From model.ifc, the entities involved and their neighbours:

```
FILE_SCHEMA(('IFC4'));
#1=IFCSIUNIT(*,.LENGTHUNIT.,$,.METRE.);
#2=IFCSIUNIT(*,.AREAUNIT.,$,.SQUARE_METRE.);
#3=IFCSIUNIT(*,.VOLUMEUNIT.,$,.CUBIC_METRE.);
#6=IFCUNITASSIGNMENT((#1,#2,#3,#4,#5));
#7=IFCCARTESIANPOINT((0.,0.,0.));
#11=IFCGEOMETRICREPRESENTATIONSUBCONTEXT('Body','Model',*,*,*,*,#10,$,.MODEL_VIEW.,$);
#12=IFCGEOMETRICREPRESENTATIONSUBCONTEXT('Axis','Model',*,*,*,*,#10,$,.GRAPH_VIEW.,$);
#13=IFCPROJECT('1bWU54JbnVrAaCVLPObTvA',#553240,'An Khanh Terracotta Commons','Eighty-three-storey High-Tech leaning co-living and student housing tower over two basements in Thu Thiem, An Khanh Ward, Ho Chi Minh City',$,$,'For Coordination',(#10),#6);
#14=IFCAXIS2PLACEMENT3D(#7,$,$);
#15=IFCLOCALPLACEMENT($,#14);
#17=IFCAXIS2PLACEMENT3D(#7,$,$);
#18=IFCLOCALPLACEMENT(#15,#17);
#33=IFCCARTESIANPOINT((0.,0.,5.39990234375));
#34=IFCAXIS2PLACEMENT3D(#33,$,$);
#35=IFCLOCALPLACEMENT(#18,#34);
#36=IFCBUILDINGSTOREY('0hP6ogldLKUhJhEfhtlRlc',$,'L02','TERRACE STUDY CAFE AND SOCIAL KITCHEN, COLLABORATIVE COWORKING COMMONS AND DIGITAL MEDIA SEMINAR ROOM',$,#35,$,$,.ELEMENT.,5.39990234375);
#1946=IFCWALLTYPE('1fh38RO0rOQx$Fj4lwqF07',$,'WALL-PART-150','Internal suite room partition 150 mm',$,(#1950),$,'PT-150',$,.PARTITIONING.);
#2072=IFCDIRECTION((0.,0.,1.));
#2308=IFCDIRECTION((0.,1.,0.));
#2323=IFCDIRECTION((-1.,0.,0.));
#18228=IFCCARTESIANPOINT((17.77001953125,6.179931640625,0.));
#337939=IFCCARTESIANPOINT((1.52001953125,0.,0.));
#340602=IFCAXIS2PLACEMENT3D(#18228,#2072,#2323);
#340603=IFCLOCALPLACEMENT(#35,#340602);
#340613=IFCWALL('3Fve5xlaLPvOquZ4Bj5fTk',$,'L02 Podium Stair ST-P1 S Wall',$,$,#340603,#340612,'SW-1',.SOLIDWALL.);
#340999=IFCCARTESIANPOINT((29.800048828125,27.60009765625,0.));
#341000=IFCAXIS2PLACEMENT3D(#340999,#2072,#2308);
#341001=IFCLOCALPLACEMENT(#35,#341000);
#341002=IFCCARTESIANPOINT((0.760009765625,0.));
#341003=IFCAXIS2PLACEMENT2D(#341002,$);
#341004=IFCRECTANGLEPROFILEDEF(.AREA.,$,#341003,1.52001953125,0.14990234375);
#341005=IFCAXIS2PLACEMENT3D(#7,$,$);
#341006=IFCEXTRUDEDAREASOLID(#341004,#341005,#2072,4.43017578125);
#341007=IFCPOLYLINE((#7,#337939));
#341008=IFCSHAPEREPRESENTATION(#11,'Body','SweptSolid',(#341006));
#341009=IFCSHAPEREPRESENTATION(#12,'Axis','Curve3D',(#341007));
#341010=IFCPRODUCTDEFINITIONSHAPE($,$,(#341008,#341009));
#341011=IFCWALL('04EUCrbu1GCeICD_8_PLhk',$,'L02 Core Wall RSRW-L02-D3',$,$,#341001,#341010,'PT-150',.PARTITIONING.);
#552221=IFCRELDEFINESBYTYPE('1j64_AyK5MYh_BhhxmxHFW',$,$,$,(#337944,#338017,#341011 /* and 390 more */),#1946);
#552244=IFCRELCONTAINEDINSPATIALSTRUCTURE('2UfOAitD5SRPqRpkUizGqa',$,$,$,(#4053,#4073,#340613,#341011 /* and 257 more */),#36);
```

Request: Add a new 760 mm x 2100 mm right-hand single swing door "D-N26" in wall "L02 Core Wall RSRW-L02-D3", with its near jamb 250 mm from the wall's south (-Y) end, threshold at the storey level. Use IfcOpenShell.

```python
import numpy as np
import ifcopenshell
import ifcopenshell.api.feature
import ifcopenshell.api.geometry
import ifcopenshell.api.root
import ifcopenshell.api.spatial
import ifcopenshell.geom
import ifcopenshell.util.element
import ifcopenshell.util.placement
import ifcopenshell.util.representation
import ifcopenshell.util.shape
import ifcopenshell.util.unit

model = ifcopenshell.open("model.ifc")
unit_scale = ifcopenshell.util.unit.calculate_unit_scale(model)
settings = ifcopenshell.geom.settings()


def volume(element):
    """Net volume in cubic metres, openings subtracted."""
    shape = ifcopenshell.geom.create_shape(settings, element)
    return ifcopenshell.util.shape.get_volume(shape.geometry)


wall = model.by_guid("04EUCrbu1GCeICD_8_PLhk")
storey = ifcopenshell.util.element.get_container(wall, ifc_class="IfcBuildingStorey")
context = ifcopenshell.util.representation.get_context(model, "Model", "Body", "MODEL_VIEW")
before = volume(wall)

width, height, from_end, sill = 0.76, 2.1, 0.25, 0.0  # metres

# The wall runs along its own X axis, and the end named is its -X end.
wall_shape = ifcopenshell.geom.create_shape(settings, wall)
x, y, z = ifcopenshell.util.shape.get_vertices(wall_shape.geometry).T
start = x.min() + from_end
face, thickness = float(y.min()), float(y.max() - y.min())
wall_matrix = ifcopenshell.util.placement.get_local_placement(wall.ObjectPlacement)
level = ifcopenshell.util.placement.get_local_placement(storey.ObjectPlacement)[2, 3]


def in_wall(x, y):
    """Placement at x, y metres in the wall's axes, at sill height."""
    matrix = wall_matrix.copy()
    matrix[:, 3] = wall_matrix @ np.array([x / unit_scale, y / unit_scale, 0.0, 1.0])
    matrix[2, 3] = level + sill / unit_scale
    return matrix


# Opening: a box that overshoots both wall faces by 50 mm.
opening = ifcopenshell.api.root.create_entity(model, ifc_class="IfcOpeningElement", predefined_type="OPENING")
box = ifcopenshell.api.geometry.add_wall_representation(
    model, context=context, length=width, height=height, thickness=thickness + 0.1
)
ifcopenshell.api.geometry.assign_representation(model, product=opening, representation=box)
ifcopenshell.api.geometry.edit_object_placement(model, product=opening, matrix=in_wall(start, face - 0.05), is_si=False)
ifcopenshell.api.feature.add_feature(model, feature=opening, element=wall)

door = ifcopenshell.api.root.create_entity(model, ifc_class="IfcDoor", name="D-N26", predefined_type="DOOR")
door.OverallWidth, door.OverallHeight = width / unit_scale, height / unit_scale
door.OperationType = "SINGLE_SWING_RIGHT"
body = ifcopenshell.api.geometry.add_door_representation(
    model,
    context=context,
    overall_width=door.OverallWidth,
    overall_height=door.OverallHeight,
    operation_type="SINGLE_SWING_RIGHT",
    lining_properties={"LiningDepth": thickness / unit_scale, "ThresholdDepth": thickness / unit_scale},
)
ifcopenshell.api.geometry.assign_representation(model, product=door, representation=body)
ifcopenshell.api.spatial.assign_container(model, products=[door], relating_structure=storey)
ifcopenshell.api.feature.add_filling(model, opening=opening, element=door)

# The lining spans the wall, so the door starts at the wall face.
ifcopenshell.api.geometry.edit_object_placement(model, product=door, matrix=in_wall(start, face), is_si=False)

after = volume(wall)

print(f"wall volume {before:.3f} -> {after:.3f} m3")

model.write("model-out.ifc")
```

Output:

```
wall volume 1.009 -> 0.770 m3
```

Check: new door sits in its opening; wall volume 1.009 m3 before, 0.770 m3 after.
